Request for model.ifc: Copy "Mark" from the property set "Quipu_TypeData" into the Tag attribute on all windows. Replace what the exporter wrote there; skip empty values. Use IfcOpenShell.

First a look at what the model holds.

```python
import ifcopenshell
import ifcopenshell.util.element

model = ifcopenshell.open("model.ifc")
print(model.schema)
windows = model.by_type("IfcWindow")
print(len(windows), "windows")
for e in windows[:8]:
    source = ifcopenshell.util.element.get_pset(e, "Quipu_TypeData", "Mark")
    target = e.Tag
    print(e.id(), repr(source), repr(target), sep=" | ")
```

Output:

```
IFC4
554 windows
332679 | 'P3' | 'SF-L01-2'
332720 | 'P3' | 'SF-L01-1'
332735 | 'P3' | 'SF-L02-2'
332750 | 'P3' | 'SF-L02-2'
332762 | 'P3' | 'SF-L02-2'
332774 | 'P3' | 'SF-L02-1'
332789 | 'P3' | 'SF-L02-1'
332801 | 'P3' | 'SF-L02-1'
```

```python
import ifcopenshell
import ifcopenshell.util.element

model = ifcopenshell.open("model.ifc")

count = 0
for e in model.by_type("IfcWindow"):
    value = ifcopenshell.util.element.get_pset(e, "Quipu_TypeData", "Mark")
    current = e.Tag
    if not value or not value.strip() or current == value:
        continue
    e.Tag = value
    count += 1

print(count, "windows updated")

model.write("model_edited.ifc")
```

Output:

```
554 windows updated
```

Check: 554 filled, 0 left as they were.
